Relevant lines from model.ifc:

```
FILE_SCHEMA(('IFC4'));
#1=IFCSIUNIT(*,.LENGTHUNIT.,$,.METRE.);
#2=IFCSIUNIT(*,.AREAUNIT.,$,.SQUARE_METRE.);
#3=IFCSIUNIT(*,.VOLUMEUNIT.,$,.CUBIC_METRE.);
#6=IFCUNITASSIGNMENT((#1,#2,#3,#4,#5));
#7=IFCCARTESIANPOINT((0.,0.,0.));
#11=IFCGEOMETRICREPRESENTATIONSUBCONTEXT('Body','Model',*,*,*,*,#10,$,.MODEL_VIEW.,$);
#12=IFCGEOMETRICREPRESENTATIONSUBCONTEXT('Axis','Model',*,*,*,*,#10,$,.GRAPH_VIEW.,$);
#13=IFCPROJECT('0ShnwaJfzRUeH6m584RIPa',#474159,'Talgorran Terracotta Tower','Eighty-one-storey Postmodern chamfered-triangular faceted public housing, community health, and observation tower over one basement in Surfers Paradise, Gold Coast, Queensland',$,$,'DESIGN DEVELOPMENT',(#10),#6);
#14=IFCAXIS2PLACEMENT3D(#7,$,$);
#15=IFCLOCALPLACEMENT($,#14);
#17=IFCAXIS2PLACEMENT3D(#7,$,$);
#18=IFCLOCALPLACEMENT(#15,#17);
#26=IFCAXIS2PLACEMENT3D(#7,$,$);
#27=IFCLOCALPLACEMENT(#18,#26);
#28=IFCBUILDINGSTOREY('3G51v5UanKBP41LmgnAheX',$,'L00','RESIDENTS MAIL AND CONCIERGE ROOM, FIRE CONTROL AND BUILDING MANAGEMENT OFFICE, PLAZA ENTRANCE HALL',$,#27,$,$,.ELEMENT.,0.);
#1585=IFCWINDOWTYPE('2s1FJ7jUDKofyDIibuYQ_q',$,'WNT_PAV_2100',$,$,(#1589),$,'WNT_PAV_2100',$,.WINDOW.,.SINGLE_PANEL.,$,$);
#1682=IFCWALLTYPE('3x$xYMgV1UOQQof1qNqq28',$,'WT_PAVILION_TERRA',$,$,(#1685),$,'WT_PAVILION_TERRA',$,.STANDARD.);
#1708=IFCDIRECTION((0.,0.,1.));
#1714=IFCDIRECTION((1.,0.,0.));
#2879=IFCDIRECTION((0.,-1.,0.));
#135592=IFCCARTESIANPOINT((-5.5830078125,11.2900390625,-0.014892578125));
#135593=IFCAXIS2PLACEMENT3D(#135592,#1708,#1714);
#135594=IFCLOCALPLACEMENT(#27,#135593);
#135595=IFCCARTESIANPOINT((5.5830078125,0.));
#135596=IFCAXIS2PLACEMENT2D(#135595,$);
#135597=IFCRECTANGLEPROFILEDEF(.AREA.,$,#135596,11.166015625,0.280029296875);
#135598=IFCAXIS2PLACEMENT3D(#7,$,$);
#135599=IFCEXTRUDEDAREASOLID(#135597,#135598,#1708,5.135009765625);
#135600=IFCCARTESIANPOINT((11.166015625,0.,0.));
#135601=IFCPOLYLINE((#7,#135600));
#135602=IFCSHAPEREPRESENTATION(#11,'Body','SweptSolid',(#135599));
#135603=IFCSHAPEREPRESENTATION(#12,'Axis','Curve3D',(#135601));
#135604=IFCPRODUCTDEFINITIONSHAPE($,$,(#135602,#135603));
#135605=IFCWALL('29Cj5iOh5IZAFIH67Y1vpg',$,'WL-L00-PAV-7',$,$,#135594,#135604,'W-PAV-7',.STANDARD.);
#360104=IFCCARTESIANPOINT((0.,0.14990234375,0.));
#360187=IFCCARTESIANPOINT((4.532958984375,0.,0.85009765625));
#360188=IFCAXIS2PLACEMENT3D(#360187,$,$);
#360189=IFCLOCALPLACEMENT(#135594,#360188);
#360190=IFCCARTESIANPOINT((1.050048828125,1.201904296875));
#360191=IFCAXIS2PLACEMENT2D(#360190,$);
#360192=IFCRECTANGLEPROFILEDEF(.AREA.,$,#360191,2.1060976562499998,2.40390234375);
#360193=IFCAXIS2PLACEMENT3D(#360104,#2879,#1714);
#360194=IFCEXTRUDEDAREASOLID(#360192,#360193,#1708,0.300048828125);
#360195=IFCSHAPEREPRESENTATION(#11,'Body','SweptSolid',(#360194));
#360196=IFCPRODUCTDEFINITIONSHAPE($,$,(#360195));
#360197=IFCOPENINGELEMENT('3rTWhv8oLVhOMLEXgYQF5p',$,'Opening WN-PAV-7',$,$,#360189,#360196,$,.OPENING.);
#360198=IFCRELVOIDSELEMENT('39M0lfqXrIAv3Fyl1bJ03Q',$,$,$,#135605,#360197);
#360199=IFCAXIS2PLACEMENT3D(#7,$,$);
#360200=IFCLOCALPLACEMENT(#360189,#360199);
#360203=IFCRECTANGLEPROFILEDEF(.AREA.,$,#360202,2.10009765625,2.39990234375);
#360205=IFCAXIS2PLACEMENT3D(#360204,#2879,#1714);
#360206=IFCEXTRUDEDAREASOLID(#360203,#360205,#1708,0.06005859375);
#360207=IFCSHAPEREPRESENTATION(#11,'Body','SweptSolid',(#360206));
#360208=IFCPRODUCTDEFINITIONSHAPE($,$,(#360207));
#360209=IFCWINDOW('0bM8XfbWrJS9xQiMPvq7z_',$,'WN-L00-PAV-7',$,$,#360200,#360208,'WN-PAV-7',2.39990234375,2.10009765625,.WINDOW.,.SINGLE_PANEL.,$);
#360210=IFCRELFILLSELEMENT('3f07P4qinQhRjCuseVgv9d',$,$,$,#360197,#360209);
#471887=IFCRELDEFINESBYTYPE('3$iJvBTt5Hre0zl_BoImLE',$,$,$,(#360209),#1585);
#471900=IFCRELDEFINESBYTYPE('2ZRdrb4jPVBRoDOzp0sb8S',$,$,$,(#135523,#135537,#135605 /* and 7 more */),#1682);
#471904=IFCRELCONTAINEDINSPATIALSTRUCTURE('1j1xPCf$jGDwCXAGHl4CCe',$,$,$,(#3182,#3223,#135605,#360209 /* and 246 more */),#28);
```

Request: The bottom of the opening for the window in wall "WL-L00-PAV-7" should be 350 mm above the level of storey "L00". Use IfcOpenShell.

```python
import numpy as np
import ifcopenshell
import ifcopenshell.api.geometry
import ifcopenshell.geom
import ifcopenshell.util.element
import ifcopenshell.util.placement
import ifcopenshell.util.shape
import ifcopenshell.util.unit

model = ifcopenshell.open("model.ifc")
unit_scale = ifcopenshell.util.unit.calculate_unit_scale(model)

window = model.by_id(360209)
opening = window.FillsVoids[0].RelatingOpeningElement
storey = ifcopenshell.util.element.get_container(window, ifc_class="IfcBuildingStorey")
level = ifcopenshell.util.placement.get_local_placement(storey.ObjectPlacement)[2, 3]

# The opening's origin need not be at the sill, so measure its lowest point.
shape = ifcopenshell.geom.create_shape(ifcopenshell.geom.settings(), opening)
bottom = ifcopenshell.util.shape.get_shape_bottom_elevation(shape, shape.geometry) / unit_scale
dz = level + 0.35 - bottom

shift = np.array([0.0, 0.0, dz])
# The window is placed relative to its opening, so it follows when the opening moves.
matrix = ifcopenshell.util.placement.get_local_placement(opening.ObjectPlacement)
matrix[:3, 3] += shift
ifcopenshell.api.geometry.edit_object_placement(
    model, product=opening, matrix=matrix, is_si=False, should_transform_children=True
)

print(f"moved by {dz * unit_scale:+.3f} m")

model.write("model_rev.ifc")
```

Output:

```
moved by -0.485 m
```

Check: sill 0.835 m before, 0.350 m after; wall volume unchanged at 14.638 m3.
